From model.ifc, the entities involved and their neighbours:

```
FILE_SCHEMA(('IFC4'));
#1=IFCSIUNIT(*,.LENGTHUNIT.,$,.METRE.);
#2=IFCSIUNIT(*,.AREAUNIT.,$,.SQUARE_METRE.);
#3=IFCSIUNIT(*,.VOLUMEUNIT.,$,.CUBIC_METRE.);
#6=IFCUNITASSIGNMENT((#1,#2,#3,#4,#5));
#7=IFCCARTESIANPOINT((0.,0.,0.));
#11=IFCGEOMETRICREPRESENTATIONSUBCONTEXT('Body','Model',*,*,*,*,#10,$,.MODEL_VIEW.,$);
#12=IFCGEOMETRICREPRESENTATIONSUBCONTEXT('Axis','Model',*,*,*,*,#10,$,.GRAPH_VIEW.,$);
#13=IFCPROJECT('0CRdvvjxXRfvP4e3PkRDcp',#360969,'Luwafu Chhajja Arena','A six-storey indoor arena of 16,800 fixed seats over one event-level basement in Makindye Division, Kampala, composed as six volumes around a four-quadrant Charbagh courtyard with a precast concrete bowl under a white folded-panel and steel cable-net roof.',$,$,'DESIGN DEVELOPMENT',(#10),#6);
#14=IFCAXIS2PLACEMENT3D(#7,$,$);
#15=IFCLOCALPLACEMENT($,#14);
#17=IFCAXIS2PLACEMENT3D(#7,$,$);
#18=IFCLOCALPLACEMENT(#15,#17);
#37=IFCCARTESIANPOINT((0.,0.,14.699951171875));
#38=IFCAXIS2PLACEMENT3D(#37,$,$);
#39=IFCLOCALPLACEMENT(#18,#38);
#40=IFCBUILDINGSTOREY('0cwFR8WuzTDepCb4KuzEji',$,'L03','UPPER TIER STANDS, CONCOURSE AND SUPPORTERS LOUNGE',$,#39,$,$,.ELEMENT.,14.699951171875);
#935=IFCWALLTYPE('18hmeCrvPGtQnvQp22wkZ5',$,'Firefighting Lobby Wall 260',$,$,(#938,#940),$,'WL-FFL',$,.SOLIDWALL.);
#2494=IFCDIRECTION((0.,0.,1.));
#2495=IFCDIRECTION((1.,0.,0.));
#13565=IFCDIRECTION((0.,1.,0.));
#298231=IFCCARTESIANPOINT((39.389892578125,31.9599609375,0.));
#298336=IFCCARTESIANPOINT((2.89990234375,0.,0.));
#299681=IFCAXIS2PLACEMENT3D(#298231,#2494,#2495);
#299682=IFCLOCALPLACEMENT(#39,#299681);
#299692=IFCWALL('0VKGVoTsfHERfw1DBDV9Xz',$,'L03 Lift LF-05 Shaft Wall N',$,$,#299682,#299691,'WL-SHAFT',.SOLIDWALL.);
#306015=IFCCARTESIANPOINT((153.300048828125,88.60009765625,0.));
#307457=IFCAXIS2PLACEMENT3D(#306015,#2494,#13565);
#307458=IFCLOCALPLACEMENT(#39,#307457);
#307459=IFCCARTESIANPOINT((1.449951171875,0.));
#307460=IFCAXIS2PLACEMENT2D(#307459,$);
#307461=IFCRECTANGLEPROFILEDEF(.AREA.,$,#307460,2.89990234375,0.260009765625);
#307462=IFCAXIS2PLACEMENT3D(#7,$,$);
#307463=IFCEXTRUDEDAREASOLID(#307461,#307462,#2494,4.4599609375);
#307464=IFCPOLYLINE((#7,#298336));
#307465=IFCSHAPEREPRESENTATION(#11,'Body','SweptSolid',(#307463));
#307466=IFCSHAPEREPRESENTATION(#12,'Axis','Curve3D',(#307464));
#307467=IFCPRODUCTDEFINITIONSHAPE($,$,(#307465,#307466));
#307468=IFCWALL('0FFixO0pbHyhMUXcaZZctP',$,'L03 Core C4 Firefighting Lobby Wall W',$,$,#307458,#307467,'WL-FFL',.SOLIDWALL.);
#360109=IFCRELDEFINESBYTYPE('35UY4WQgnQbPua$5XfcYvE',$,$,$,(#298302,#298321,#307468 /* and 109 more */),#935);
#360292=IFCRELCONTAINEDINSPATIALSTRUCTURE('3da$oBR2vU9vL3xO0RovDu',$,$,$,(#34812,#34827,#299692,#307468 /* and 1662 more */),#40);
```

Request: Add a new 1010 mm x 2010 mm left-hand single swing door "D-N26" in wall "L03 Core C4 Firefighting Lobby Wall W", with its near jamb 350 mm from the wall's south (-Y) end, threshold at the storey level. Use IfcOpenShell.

```python
import numpy as np
import ifcopenshell
import ifcopenshell.api.feature
import ifcopenshell.api.geometry
import ifcopenshell.api.root
import ifcopenshell.api.spatial
import ifcopenshell.geom
import ifcopenshell.util.element
import ifcopenshell.util.placement
import ifcopenshell.util.representation
import ifcopenshell.util.shape
import ifcopenshell.util.unit

model = ifcopenshell.open("model.ifc")
unit_scale = ifcopenshell.util.unit.calculate_unit_scale(model)
settings = ifcopenshell.geom.settings()


def volume(element):
    """Net volume in cubic metres, openings subtracted."""
    shape = ifcopenshell.geom.create_shape(settings, element)
    return ifcopenshell.util.shape.get_volume(shape.geometry)


wall = model.by_guid("0FFixO0pbHyhMUXcaZZctP")
storey = ifcopenshell.util.element.get_container(wall, ifc_class="IfcBuildingStorey")
context = ifcopenshell.util.representation.get_context(model, "Model", "Body", "MODEL_VIEW")
before = volume(wall)

width, height, from_end, sill = 1.01, 2.01, 0.35, 0.0  # metres

# The wall runs along its own X axis, and the end named is its -X end.
wall_shape = ifcopenshell.geom.create_shape(settings, wall)
x, y, z = ifcopenshell.util.shape.get_vertices(wall_shape.geometry).T
start = x.min() + from_end
face, thickness = float(y.min()), float(y.max() - y.min())
wall_matrix = ifcopenshell.util.placement.get_local_placement(wall.ObjectPlacement)
level = ifcopenshell.util.placement.get_local_placement(storey.ObjectPlacement)[2, 3]


def in_wall(x, y):
    """Placement at x, y metres in the wall's axes, at sill height."""
    matrix = wall_matrix.copy()
    matrix[:, 3] = wall_matrix @ np.array([x / unit_scale, y / unit_scale, 0.0, 1.0])
    matrix[2, 3] = level + sill / unit_scale
    return matrix


# Opening: a box that overshoots both wall faces by 50 mm.
opening = ifcopenshell.api.root.create_entity(model, ifc_class="IfcOpeningElement", predefined_type="OPENING")
box = ifcopenshell.api.geometry.add_wall_representation(
    model, context=context, length=width, height=height, thickness=thickness + 0.1
)
ifcopenshell.api.geometry.assign_representation(model, product=opening, representation=box)
ifcopenshell.api.geometry.edit_object_placement(model, product=opening, matrix=in_wall(start, face - 0.05), is_si=False)
ifcopenshell.api.feature.add_feature(model, feature=opening, element=wall)

door = ifcopenshell.api.root.create_entity(model, ifc_class="IfcDoor", name="D-N26", predefined_type="DOOR")
door.OverallWidth, door.OverallHeight = width / unit_scale, height / unit_scale
door.OperationType = "SINGLE_SWING_LEFT"
body = ifcopenshell.api.geometry.add_door_representation(
    model,
    context=context,
    overall_width=door.OverallWidth,
    overall_height=door.OverallHeight,
    operation_type="SINGLE_SWING_LEFT",
    lining_properties={"LiningDepth": thickness / unit_scale, "ThresholdDepth": thickness / unit_scale},
)
ifcopenshell.api.geometry.assign_representation(model, product=door, representation=body)
ifcopenshell.api.spatial.assign_container(model, products=[door], relating_structure=storey)
ifcopenshell.api.feature.add_filling(model, opening=opening, element=door)

# The lining spans the wall, so the door starts at the wall face.
ifcopenshell.api.geometry.edit_object_placement(model, product=door, matrix=in_wall(start, face), is_si=False)

after = volume(wall)

print(f"wall volume {before:.3f} -> {after:.3f} m3")

model.write("model_rev.ifc")
```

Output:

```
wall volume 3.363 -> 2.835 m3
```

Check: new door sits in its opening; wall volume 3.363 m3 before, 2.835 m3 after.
